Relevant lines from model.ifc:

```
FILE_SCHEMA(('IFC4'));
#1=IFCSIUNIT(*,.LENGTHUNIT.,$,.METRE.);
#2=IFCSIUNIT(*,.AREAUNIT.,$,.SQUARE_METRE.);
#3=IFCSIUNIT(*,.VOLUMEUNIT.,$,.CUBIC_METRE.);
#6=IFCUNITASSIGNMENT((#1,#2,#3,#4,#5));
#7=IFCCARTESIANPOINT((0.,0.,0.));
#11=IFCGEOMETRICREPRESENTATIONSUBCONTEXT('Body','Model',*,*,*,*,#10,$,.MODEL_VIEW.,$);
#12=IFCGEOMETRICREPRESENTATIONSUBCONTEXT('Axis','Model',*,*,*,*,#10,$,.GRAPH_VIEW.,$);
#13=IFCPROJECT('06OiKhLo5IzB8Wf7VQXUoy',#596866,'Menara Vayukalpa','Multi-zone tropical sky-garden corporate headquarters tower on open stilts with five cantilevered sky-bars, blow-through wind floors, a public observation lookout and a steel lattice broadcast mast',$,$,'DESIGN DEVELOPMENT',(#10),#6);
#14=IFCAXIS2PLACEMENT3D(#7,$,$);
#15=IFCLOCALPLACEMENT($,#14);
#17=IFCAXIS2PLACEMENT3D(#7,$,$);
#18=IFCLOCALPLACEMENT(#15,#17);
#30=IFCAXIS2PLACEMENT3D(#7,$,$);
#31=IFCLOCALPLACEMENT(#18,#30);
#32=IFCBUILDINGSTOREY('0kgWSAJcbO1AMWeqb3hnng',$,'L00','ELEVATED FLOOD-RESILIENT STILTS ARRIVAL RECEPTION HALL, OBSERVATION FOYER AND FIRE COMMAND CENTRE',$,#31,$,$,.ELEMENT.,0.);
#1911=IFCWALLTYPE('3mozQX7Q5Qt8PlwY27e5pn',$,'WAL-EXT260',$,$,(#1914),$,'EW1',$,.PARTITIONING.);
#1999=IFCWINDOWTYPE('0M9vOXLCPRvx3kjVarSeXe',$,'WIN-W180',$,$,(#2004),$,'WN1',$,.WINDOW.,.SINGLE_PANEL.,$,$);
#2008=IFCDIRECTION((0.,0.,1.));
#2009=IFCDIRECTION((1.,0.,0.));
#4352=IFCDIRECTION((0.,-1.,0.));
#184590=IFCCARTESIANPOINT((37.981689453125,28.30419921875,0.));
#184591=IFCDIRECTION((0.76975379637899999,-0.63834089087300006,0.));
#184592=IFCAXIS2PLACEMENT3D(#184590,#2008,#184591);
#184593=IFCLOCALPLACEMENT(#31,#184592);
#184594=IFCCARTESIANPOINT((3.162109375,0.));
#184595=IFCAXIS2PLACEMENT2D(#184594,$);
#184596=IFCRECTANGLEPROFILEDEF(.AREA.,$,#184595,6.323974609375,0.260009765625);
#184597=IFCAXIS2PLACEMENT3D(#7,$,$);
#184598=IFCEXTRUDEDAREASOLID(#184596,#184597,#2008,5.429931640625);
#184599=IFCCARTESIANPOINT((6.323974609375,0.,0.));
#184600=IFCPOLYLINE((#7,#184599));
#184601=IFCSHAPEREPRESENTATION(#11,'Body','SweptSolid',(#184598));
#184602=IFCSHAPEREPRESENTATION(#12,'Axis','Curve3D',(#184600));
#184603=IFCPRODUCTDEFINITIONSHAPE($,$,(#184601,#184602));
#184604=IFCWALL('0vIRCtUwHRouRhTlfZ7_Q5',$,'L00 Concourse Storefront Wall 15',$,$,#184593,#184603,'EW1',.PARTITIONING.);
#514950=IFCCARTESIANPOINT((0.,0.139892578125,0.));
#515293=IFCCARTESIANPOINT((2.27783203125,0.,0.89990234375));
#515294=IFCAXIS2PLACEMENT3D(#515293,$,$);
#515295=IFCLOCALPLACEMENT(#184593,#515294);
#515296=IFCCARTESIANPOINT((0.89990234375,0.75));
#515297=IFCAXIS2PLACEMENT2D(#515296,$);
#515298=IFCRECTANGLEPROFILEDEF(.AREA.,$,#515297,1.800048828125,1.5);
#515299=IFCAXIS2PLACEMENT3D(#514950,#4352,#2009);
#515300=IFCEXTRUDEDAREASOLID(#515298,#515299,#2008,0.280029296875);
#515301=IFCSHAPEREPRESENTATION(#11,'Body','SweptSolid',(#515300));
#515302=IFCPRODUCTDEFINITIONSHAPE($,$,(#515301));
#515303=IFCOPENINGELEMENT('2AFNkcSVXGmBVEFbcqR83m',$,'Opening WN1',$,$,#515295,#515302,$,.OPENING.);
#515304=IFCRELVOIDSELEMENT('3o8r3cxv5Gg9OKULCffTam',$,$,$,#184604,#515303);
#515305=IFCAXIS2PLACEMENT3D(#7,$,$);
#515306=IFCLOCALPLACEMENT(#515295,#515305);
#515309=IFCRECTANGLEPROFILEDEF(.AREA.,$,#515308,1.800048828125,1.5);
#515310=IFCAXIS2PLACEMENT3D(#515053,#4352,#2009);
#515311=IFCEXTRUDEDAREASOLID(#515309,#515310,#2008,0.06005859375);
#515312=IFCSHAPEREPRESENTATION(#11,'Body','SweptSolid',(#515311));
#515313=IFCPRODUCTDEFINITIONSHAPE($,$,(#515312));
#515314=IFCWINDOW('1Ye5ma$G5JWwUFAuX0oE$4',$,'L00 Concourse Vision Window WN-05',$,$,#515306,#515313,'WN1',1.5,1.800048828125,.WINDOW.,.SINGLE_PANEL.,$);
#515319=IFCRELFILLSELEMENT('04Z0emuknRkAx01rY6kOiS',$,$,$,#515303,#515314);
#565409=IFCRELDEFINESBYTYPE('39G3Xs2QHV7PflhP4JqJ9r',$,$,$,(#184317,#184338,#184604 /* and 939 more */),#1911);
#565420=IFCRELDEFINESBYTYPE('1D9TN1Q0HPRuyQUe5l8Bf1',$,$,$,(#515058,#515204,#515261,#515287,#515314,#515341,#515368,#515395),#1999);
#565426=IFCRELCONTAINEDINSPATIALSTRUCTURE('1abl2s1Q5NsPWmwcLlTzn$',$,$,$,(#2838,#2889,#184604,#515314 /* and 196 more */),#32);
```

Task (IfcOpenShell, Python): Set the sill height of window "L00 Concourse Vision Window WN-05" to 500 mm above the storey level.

```python
import numpy as np
import ifcopenshell
import ifcopenshell.api.geometry
import ifcopenshell.geom
import ifcopenshell.util.element
import ifcopenshell.util.placement
import ifcopenshell.util.shape
import ifcopenshell.util.unit

model = ifcopenshell.open("model.ifc")
unit_scale = ifcopenshell.util.unit.calculate_unit_scale(model)

window = model.by_guid("1Ye5ma$G5JWwUFAuX0oE$4")
opening = window.FillsVoids[0].RelatingOpeningElement
storey = ifcopenshell.util.element.get_container(window, ifc_class="IfcBuildingStorey")
level = ifcopenshell.util.placement.get_local_placement(storey.ObjectPlacement)[2, 3]

# The opening's origin need not be at the sill, so measure its lowest point.
shape = ifcopenshell.geom.create_shape(ifcopenshell.geom.settings(), opening)
bottom = ifcopenshell.util.shape.get_shape_bottom_elevation(shape, shape.geometry) / unit_scale
dz = level + 0.5 / unit_scale - bottom

shift = np.array([0.0, 0.0, dz])
# The window is placed relative to its opening, so it follows when the opening moves.
matrix = ifcopenshell.util.placement.get_local_placement(opening.ObjectPlacement)
matrix[:3, 3] += shift
ifcopenshell.api.geometry.edit_object_placement(
    model, product=opening, matrix=matrix, is_si=False, should_transform_children=True
)

print(f"moved by {dz * unit_scale:+.3f} m")

model.write("model_edited.ifc")
```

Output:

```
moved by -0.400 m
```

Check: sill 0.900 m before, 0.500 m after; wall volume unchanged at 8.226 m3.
